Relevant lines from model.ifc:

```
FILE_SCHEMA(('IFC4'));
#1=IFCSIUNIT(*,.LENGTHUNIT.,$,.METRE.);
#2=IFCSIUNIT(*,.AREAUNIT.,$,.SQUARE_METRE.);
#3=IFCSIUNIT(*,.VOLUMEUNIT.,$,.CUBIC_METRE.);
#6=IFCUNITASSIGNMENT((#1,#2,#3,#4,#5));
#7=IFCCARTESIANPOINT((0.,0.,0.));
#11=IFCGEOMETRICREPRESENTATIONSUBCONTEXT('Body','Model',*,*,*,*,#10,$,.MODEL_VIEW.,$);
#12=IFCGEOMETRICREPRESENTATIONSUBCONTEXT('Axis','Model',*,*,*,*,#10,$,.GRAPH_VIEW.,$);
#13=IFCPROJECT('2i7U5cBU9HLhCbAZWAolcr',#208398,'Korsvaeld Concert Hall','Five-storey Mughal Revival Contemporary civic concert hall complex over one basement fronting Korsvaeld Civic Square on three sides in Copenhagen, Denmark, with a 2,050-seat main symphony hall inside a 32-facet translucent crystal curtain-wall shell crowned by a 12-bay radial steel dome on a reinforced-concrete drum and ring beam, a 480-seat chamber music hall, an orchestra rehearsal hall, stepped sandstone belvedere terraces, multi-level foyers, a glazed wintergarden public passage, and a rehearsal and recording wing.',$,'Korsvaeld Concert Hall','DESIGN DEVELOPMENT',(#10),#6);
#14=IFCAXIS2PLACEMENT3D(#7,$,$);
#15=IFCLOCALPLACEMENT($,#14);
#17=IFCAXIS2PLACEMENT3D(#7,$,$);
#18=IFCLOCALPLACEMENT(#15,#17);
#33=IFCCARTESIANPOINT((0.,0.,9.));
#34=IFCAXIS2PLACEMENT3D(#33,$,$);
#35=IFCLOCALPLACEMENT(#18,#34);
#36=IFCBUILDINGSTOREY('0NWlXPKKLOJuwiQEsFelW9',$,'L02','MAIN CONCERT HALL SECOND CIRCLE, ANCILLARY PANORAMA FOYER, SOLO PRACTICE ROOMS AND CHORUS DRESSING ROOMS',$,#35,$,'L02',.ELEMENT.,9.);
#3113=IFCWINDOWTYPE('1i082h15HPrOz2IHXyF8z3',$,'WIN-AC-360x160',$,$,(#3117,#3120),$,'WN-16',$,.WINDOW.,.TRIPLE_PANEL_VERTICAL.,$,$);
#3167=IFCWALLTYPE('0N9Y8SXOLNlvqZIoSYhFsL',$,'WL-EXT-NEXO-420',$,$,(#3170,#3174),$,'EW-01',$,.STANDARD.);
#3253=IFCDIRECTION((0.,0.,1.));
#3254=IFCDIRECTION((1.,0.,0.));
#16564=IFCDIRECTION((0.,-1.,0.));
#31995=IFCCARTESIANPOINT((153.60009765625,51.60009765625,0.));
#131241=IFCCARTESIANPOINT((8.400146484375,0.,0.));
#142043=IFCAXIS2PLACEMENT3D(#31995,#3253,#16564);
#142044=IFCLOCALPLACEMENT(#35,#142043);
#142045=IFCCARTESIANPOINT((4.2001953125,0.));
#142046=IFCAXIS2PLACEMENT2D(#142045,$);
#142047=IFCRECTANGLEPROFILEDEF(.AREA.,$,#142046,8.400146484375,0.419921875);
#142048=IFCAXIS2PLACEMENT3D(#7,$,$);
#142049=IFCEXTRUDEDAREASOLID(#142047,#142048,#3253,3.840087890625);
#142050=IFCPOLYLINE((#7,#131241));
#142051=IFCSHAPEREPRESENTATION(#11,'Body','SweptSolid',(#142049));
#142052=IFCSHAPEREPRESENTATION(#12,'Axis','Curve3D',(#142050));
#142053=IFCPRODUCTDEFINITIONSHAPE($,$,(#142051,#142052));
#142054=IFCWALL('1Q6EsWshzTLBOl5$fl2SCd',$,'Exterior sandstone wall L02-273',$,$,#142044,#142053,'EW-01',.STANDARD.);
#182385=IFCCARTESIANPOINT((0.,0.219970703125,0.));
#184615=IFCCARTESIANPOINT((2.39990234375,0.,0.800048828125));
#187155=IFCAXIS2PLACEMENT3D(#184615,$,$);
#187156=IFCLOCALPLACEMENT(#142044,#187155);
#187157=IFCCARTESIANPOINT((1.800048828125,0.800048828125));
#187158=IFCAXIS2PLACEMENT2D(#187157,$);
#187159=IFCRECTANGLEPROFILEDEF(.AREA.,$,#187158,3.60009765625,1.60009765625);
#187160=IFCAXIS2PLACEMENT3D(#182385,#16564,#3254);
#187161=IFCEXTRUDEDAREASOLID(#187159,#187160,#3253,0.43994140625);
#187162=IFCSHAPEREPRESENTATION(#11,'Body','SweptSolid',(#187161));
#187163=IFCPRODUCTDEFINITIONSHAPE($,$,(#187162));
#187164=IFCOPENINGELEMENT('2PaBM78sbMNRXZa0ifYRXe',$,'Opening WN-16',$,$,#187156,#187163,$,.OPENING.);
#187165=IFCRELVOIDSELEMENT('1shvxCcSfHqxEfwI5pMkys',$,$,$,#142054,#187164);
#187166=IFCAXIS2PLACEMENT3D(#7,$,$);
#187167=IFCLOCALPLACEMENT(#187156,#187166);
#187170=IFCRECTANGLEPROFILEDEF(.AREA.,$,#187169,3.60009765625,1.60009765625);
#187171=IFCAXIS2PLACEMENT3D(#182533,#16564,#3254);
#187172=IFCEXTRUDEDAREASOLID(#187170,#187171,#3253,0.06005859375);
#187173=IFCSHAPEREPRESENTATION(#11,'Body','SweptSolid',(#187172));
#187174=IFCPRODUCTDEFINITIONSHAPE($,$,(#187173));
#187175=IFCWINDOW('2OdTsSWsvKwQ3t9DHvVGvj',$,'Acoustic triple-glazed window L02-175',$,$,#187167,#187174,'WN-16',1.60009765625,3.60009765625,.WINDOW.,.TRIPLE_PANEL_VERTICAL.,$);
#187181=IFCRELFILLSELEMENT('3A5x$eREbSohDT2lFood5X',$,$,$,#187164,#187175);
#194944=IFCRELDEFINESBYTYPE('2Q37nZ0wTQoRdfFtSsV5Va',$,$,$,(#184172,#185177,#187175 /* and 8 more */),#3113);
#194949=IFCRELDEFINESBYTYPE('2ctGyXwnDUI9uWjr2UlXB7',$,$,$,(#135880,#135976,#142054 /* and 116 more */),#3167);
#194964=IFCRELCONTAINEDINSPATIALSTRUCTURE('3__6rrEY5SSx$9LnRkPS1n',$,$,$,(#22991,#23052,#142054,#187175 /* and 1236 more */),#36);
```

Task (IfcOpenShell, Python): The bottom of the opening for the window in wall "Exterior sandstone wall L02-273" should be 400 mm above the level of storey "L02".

```python
import numpy as np
import ifcopenshell
import ifcopenshell.api.geometry
import ifcopenshell.geom
import ifcopenshell.util.element
import ifcopenshell.util.placement
import ifcopenshell.util.shape
import ifcopenshell.util.unit

model = ifcopenshell.open("model.ifc")
unit_scale = ifcopenshell.util.unit.calculate_unit_scale(model)

window = model.by_id(187175)
opening = window.FillsVoids[0].RelatingOpeningElement
storey = ifcopenshell.util.element.get_container(window, ifc_class="IfcBuildingStorey")
level = ifcopenshell.util.placement.get_local_placement(storey.ObjectPlacement)[2, 3]

# The opening's origin need not be at the sill, so measure its lowest point.
shape = ifcopenshell.geom.create_shape(ifcopenshell.geom.settings(), opening)
bottom = ifcopenshell.util.shape.get_shape_bottom_elevation(shape, shape.geometry) / unit_scale
dz = level + 0.4 / unit_scale - bottom

shift = np.array([0.0, 0.0, dz])
# The window is placed relative to its opening, so it follows when the opening moves.
matrix = ifcopenshell.util.placement.get_local_placement(opening.ObjectPlacement)
matrix[:3, 3] += shift
ifcopenshell.api.geometry.edit_object_placement(
    model, product=opening, matrix=matrix, is_si=False, should_transform_children=True
)

print(f"moved by {dz * unit_scale:+.3f} m")

model.write("model_rev.ifc")
```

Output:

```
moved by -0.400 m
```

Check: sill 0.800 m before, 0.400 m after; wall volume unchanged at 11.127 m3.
